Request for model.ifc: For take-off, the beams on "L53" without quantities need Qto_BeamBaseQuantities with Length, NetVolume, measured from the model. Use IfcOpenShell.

First a look at what the model holds.

```python
import ifcopenshell
import ifcopenshell.util.element
import ifcopenshell.util.unit

model = ifcopenshell.open("model.ifc")
print(model.schema)
for unit_type in ("LENGTHUNIT", "AREAUNIT", "VOLUMEUNIT"):
    print(unit_type, ifcopenshell.util.unit.calculate_unit_scale(model, unit_type))
storey = next(s for s in model.by_type("IfcBuildingStorey") if s.Name == "L53")
beams = [e for e in ifcopenshell.util.element.get_decomposition(storey) if e.is_a("IfcBeam")]
for e in sorted(beams, key=lambda e: e.id()):
    print(e.id(), e.is_a(), e.Name, list(ifcopenshell.util.element.get_psets(e, qtos_only=True)), sep=" | ")
```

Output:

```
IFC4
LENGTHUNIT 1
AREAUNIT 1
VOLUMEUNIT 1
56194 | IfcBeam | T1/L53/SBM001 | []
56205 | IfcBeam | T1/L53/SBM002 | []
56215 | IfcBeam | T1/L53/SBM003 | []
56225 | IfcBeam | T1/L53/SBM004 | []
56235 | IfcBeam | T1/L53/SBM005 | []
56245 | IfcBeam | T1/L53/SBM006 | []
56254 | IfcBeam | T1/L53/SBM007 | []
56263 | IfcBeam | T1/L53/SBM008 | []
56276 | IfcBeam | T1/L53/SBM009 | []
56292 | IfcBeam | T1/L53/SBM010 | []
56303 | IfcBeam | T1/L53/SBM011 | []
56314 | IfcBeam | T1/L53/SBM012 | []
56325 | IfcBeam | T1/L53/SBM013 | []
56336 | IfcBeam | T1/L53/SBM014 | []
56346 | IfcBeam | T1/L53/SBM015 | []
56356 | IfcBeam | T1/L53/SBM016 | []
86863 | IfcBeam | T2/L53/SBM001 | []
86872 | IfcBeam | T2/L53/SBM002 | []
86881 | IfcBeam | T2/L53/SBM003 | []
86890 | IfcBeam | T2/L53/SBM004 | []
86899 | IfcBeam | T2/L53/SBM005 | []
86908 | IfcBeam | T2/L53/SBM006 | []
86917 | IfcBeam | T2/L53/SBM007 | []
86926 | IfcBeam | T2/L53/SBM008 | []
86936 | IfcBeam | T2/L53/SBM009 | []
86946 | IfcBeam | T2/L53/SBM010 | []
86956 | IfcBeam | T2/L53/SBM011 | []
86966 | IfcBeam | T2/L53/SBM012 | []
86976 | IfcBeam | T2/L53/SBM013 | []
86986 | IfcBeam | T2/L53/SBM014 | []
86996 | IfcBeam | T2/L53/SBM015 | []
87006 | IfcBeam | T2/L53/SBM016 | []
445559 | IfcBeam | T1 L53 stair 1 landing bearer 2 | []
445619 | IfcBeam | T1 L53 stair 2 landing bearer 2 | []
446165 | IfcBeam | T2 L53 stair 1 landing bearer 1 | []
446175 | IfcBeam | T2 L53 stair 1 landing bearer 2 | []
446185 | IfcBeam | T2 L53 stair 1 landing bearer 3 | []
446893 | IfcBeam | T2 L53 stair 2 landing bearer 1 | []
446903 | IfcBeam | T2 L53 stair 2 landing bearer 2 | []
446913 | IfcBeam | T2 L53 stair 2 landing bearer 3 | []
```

```python
import ifcopenshell
import ifcopenshell.api.pset
import ifcopenshell.geom
import ifcopenshell.util.element
import ifcopenshell.util.shape
import ifcopenshell.util.unit

model = ifcopenshell.open("model.ifc")
unit_scale = ifcopenshell.util.unit.calculate_unit_scale(model)
volume_scale = ifcopenshell.util.unit.calculate_unit_scale(model, "VOLUMEUNIT")
settings = ifcopenshell.geom.settings()

storey = next(s for s in model.by_type("IfcBuildingStorey") if s.Name == "L53")
beams = [e for e in ifcopenshell.util.element.get_decomposition(storey) if e.is_a("IfcBeam")]

for e in sorted(beams, key=lambda e: e.id()):
    if ifcopenshell.util.element.get_psets(e, qtos_only=True, should_inherit=False):
        continue
    # Geometry comes back in metres, in the element's own axes.
    shape = ifcopenshell.geom.create_shape(settings, e)
    values = {
        "Length": ifcopenshell.util.shape.get_max_xyz(shape.geometry) / unit_scale,
        "NetVolume": ifcopenshell.util.shape.get_volume(shape.geometry) / volume_scale,
    }
    qto = ifcopenshell.api.pset.add_qto(model, product=e, name="Qto_BeamBaseQuantities")
    ifcopenshell.api.pset.edit_qto(model, qto=qto, properties=values)
    print(e.id(), {k: round(v, 3) for k, v in values.items()})

model.write("model-out.ifc")
```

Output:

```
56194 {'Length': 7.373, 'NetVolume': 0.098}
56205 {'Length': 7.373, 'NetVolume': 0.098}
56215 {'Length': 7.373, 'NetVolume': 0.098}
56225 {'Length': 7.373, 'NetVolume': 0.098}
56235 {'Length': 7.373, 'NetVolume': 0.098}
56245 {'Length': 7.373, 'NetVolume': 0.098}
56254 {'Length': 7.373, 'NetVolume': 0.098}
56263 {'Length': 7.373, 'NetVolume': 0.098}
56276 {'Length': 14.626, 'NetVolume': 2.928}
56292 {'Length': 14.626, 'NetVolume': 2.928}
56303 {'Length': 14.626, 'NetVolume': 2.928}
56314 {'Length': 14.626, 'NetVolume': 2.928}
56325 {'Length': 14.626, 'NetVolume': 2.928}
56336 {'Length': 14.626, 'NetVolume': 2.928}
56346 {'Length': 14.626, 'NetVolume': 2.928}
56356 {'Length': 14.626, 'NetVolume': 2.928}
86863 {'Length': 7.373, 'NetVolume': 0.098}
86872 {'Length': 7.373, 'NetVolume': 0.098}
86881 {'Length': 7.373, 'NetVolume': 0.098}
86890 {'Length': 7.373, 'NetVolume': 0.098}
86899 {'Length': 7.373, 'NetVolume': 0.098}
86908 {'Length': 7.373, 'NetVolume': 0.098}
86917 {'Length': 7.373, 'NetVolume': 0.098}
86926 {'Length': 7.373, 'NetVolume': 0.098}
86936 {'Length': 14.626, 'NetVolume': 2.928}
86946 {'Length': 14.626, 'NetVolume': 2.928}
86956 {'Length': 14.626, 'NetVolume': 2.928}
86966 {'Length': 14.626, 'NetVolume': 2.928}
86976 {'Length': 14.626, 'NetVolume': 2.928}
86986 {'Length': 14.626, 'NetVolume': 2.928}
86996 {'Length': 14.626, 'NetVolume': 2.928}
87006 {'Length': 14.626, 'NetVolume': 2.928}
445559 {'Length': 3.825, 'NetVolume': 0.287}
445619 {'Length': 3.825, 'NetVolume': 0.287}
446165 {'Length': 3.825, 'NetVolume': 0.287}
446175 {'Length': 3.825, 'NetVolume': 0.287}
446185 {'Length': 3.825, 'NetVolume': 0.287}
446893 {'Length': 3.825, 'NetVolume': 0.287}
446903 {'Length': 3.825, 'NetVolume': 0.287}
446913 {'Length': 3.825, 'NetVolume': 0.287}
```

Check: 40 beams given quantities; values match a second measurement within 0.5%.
